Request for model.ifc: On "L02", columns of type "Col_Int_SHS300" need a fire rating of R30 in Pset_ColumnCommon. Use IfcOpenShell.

First a look at what the model holds.

```python
import ifcopenshell
import ifcopenshell.util.element

model = ifcopenshell.open("model.ifc")
print(model.schema)
storey = next(s for s in model.by_type("IfcBuildingStorey") if s.Name == "L02")
columns = [e for e in ifcopenshell.util.element.get_decomposition(storey) if e.is_a("IfcColumn")]
seen = {}
for e in columns:
    element_type = ifcopenshell.util.element.get_type(e)
    key = (element_type.Name if element_type != e and element_type else None, ifcopenshell.util.element.get_pset(e, "Pset_ColumnCommon", "FireRating"))
    seen[key] = seen.get(key, 0) + 1
for (name, value), count in sorted(seen.items(), key=str):
    print(count, "x", name, "|", value)
```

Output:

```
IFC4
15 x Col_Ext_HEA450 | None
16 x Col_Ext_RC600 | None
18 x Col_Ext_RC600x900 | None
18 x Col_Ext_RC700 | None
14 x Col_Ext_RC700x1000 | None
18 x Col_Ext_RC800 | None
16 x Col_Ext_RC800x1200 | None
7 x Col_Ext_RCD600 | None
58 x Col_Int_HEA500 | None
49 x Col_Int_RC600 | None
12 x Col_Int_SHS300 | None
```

```python
import ifcopenshell
import ifcopenshell.api.pset
import ifcopenshell.util.element

model = ifcopenshell.open("model.ifc")

storey = next(s for s in model.by_type("IfcBuildingStorey") if s.Name == "L02")
columns = [e for e in ifcopenshell.util.element.get_decomposition(storey) if e.is_a("IfcColumn")]

count = 0
for e in columns:
    element_type = ifcopenshell.util.element.get_type(e)
    if element_type in (None, e) or element_type.Name != "Col_Int_SHS300":
        continue
    # add_pset returns the element's existing set when there is one.
    pset = ifcopenshell.api.pset.add_pset(model, product=e, name="Pset_ColumnCommon")
    ifcopenshell.api.pset.edit_pset(model, pset=pset, properties={"FireRating": "R30"})
    count += 1

print(count, "columns updated")

model.write("model_rev.ifc")
```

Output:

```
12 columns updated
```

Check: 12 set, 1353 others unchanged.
